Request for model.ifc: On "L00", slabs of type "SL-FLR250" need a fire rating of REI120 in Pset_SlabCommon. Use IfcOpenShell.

First a look at what the model holds.

```python
import ifcopenshell
import ifcopenshell.util.element

model = ifcopenshell.open("model.ifc")
print(model.schema)
storey = next(s for s in model.by_type("IfcBuildingStorey") if s.Name == "L00")
slabs = [e for e in ifcopenshell.util.element.get_decomposition(storey) if e.is_a("IfcSlab")]
seen = {}
for e in slabs:
    element_type = ifcopenshell.util.element.get_type(e)
    key = (element_type.Name if element_type != e and element_type else None, ifcopenshell.util.element.get_pset(e, "Pset_SlabCommon", "FireRating"))
    seen[key] = seen.get(key, 0) + 1
for (name, value), count in sorted(seen.items(), key=str):
    print(count, "x", name, "|", value)
```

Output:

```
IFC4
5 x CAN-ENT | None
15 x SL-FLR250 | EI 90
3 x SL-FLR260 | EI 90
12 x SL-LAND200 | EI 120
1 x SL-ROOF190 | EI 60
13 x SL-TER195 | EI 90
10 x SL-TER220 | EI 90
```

```python
import ifcopenshell
import ifcopenshell.api.pset
import ifcopenshell.util.element

model = ifcopenshell.open("model.ifc")

storey = next(s for s in model.by_type("IfcBuildingStorey") if s.Name == "L00")
slabs = [e for e in ifcopenshell.util.element.get_decomposition(storey) if e.is_a("IfcSlab")]

count = 0
for e in slabs:
    element_type = ifcopenshell.util.element.get_type(e)
    if element_type in (None, e) or element_type.Name != "SL-FLR250":
        continue
    # add_pset returns the element's existing set when there is one.
    pset = ifcopenshell.api.pset.add_pset(model, product=e, name="Pset_SlabCommon")
    ifcopenshell.api.pset.edit_pset(model, pset=pset, properties={"FireRating": "REI120"})
    count += 1

print(count, "slabs updated")

model.write("model-out.ifc")
```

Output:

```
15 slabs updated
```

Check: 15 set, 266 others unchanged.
